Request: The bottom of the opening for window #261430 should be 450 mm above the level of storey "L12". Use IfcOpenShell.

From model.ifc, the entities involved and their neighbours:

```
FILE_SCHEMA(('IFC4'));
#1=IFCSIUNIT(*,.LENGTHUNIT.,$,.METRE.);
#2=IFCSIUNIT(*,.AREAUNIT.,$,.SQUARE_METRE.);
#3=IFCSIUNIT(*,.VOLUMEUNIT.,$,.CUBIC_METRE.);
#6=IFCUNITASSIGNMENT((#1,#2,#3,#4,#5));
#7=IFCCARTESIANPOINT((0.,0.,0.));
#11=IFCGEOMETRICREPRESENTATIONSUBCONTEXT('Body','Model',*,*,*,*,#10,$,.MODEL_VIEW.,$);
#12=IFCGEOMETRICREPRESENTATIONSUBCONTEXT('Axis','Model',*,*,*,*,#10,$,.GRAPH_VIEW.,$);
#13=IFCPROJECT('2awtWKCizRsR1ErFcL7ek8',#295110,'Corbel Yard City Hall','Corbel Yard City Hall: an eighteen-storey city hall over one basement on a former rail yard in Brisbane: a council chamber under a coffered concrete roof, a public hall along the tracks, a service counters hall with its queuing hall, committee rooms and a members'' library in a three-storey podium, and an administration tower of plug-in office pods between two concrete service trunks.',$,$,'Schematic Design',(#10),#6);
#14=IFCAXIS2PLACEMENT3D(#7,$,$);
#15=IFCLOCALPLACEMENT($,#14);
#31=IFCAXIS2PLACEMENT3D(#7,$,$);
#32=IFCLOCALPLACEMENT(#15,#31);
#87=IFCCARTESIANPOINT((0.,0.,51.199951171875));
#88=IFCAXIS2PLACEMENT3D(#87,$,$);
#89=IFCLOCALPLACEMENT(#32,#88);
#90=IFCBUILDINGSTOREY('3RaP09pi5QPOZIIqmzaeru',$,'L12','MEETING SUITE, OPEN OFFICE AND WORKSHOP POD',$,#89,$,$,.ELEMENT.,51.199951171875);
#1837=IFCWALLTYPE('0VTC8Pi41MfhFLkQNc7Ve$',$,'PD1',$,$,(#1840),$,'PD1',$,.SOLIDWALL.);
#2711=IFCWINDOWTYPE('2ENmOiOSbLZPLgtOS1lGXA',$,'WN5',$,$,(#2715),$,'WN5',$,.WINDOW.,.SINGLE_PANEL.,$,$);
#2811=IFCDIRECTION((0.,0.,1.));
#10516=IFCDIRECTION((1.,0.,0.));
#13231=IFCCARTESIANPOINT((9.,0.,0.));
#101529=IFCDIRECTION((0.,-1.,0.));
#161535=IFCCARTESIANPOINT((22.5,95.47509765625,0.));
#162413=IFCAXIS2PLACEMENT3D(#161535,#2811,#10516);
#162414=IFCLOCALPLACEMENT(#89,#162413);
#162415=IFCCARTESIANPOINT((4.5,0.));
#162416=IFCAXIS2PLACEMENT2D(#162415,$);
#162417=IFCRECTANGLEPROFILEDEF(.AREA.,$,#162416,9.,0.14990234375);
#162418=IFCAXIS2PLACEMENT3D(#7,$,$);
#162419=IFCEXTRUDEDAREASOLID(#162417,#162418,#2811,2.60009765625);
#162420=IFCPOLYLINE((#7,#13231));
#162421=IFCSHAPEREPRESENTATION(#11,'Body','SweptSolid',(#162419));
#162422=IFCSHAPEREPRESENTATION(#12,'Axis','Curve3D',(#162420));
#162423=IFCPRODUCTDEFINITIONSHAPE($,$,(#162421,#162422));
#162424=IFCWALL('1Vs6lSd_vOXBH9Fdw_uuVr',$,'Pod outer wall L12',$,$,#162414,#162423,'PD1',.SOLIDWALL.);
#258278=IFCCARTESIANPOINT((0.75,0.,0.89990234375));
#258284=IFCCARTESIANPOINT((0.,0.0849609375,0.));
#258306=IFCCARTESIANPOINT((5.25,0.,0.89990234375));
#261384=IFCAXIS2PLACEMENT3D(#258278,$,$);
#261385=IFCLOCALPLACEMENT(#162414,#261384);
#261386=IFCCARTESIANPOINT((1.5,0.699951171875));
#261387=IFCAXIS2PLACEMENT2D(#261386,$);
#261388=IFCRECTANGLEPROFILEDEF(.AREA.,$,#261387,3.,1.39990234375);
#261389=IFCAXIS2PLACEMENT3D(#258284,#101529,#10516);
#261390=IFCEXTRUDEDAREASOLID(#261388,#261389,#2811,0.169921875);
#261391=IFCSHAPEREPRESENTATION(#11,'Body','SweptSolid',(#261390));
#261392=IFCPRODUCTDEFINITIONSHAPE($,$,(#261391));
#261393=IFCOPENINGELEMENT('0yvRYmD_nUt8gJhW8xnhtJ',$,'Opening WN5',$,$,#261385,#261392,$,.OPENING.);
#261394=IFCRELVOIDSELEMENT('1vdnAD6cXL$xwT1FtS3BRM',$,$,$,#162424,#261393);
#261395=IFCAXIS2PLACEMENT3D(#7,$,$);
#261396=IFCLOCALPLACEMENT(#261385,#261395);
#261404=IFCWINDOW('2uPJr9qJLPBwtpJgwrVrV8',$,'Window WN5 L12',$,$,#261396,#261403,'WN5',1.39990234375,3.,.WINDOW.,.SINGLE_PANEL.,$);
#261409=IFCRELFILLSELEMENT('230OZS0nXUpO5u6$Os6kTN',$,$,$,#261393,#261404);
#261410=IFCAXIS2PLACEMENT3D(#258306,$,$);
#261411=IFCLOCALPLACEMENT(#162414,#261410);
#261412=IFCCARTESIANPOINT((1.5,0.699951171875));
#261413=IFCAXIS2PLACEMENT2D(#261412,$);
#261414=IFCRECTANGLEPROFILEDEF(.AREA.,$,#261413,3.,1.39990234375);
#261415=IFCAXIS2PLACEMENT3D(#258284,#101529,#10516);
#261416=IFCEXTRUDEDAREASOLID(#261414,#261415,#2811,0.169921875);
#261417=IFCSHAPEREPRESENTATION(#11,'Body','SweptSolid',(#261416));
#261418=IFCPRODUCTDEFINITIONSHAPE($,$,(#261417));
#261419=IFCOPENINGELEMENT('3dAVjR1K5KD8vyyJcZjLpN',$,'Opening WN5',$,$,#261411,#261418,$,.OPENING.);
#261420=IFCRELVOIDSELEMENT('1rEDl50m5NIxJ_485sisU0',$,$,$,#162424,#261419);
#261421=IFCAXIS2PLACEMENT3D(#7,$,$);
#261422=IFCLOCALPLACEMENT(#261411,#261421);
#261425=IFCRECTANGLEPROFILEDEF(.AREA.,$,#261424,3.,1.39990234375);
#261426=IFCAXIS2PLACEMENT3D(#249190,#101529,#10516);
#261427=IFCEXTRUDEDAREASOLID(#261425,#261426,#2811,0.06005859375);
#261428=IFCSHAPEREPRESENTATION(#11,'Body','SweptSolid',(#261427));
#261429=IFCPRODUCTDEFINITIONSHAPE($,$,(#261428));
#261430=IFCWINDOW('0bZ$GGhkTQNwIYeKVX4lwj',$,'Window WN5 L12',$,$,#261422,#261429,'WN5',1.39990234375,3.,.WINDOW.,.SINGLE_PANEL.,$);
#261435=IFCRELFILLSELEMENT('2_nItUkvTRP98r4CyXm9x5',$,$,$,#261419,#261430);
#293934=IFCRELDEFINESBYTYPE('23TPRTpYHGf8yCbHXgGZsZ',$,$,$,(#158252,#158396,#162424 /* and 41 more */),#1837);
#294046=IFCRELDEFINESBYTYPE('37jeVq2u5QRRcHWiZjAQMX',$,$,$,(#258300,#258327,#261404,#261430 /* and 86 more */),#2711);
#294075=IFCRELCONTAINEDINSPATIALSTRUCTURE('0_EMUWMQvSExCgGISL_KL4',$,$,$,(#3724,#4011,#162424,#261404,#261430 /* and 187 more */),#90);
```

```python
import numpy as np
import ifcopenshell
import ifcopenshell.api.geometry
import ifcopenshell.geom
import ifcopenshell.util.element
import ifcopenshell.util.placement
import ifcopenshell.util.shape
import ifcopenshell.util.unit

model = ifcopenshell.open("model.ifc")
unit_scale = ifcopenshell.util.unit.calculate_unit_scale(model)

window = model.by_id(261430)
opening = window.FillsVoids[0].RelatingOpeningElement
storey = ifcopenshell.util.element.get_container(window, ifc_class="IfcBuildingStorey")
level = ifcopenshell.util.placement.get_local_placement(storey.ObjectPlacement)[2, 3]

# The opening's origin need not be at the sill, so measure its lowest point.
shape = ifcopenshell.geom.create_shape(ifcopenshell.geom.settings(), opening)
bottom = ifcopenshell.util.shape.get_shape_bottom_elevation(shape, shape.geometry) / unit_scale
dz = level + 0.45 - bottom

shift = np.array([0.0, 0.0, dz])
# The window is placed relative to its opening, so it follows when the opening moves.
matrix = ifcopenshell.util.placement.get_local_placement(opening.ObjectPlacement)
matrix[:3, 3] += shift
ifcopenshell.api.geometry.edit_object_placement(
    model, product=opening, matrix=matrix, is_si=False, should_transform_children=True
)

print(f"moved by {dz * unit_scale:+.3f} m")

model.write("model_updated.ifc")
```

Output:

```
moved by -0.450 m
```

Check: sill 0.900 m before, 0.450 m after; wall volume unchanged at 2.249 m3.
